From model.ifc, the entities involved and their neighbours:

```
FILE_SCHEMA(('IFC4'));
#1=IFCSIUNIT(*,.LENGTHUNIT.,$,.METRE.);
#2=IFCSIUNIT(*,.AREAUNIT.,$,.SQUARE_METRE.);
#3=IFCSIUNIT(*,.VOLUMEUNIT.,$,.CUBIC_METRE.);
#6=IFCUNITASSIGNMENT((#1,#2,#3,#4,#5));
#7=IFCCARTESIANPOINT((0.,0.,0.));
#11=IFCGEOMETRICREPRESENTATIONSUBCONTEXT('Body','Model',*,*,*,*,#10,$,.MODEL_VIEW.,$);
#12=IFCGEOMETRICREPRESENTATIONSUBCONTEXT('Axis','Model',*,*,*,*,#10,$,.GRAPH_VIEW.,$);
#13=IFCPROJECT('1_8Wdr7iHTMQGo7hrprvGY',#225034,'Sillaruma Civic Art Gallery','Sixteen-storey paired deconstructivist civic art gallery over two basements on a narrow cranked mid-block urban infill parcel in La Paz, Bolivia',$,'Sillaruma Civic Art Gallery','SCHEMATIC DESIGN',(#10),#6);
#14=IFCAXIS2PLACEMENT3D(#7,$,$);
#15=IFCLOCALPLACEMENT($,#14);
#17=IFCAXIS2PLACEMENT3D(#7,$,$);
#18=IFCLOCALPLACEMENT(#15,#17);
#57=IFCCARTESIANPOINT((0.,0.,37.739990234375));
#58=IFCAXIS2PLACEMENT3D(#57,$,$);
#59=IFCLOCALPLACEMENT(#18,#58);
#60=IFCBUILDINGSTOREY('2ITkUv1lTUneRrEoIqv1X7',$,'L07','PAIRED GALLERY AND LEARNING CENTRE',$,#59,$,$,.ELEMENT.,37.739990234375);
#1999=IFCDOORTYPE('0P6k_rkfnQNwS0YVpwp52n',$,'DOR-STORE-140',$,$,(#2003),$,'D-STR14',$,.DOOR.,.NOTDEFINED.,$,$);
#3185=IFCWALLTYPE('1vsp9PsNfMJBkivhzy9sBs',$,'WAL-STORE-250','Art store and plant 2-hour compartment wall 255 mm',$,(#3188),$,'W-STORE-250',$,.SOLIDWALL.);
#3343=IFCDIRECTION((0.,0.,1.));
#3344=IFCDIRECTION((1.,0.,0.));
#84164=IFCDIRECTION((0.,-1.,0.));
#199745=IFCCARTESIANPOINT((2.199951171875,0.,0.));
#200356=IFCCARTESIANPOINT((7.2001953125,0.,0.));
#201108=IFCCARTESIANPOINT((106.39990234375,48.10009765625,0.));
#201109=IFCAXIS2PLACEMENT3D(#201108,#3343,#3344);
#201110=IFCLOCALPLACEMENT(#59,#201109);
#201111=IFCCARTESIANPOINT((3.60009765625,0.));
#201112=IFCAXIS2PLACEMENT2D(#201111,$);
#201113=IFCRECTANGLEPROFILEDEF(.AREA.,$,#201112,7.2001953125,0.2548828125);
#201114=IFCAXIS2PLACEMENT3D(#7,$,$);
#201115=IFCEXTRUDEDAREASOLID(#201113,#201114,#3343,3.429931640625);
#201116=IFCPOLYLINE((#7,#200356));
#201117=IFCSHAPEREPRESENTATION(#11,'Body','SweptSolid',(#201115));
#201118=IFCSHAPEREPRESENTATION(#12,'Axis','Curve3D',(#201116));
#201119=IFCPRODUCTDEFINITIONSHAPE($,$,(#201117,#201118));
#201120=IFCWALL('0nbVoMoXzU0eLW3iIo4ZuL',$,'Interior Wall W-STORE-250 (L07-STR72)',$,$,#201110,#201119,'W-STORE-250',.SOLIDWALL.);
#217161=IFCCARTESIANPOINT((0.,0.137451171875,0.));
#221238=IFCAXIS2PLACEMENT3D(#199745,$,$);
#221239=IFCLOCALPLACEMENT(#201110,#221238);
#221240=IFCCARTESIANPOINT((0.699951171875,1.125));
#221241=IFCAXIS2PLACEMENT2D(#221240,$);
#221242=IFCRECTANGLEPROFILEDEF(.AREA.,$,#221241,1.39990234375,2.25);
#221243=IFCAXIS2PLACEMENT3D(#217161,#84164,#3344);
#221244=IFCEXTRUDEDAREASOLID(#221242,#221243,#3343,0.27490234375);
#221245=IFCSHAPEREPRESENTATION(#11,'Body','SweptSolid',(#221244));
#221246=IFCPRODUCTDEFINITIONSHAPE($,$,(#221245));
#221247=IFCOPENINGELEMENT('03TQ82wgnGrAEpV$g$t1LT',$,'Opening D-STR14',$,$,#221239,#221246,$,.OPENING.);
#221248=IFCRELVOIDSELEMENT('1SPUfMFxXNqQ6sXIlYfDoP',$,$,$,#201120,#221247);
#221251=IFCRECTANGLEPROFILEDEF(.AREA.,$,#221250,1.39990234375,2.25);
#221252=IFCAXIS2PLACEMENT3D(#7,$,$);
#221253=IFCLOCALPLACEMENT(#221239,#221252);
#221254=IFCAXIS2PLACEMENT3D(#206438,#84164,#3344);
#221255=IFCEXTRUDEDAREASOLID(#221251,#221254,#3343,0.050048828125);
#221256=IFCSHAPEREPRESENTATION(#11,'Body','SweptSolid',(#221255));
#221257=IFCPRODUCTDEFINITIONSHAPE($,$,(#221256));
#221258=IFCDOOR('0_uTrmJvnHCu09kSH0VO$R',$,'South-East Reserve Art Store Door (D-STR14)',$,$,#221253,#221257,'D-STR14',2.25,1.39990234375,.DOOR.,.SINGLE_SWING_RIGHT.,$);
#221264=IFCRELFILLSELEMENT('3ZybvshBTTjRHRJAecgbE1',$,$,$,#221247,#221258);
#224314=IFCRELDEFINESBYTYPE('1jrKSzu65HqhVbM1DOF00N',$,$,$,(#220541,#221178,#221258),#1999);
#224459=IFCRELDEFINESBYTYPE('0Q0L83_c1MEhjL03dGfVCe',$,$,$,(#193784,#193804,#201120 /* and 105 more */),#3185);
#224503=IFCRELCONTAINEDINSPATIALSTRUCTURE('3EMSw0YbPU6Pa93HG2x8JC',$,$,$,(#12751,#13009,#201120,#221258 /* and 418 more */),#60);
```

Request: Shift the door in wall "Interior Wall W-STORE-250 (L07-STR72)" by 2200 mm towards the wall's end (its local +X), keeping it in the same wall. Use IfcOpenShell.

```python
import ifcopenshell
import ifcopenshell.api.geometry
import ifcopenshell.util.placement

model = ifcopenshell.open("model.ifc")

door = model.by_guid("0_uTrmJvnHCu09kSH0VO$R")
opening = door.FillsVoids[0].RelatingOpeningElement
wall = opening.VoidsElements[0].RelatingBuildingElement

wall_matrix = ifcopenshell.util.placement.get_local_placement(wall.ObjectPlacement)
shift = wall_matrix[:3, 0] * 2.2
before = ifcopenshell.util.placement.get_local_placement(door.ObjectPlacement)[:3, 3].copy()

# The door is placed relative to its opening, so it follows when the opening moves.
matrix = ifcopenshell.util.placement.get_local_placement(opening.ObjectPlacement)
matrix[:3, 3] += shift
ifcopenshell.api.geometry.edit_object_placement(
    model, product=opening, matrix=matrix, is_si=False, should_transform_children=True
)

after = ifcopenshell.util.placement.get_local_placement(door.ObjectPlacement)[:3, 3]
print("door moved by", (after - before).round(3) + 0.0)

model.write("model_edited.ifc")
```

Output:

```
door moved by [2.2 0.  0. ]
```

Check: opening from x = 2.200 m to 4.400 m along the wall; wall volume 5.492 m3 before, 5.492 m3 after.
